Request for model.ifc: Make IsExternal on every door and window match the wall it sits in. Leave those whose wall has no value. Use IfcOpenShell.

First a look at what the model holds.

```python
import ifcopenshell
import ifcopenshell.util.element

model = ifcopenshell.open("model.ifc")
print(model.schema)
seen = {}
for e in model.by_type("IfcDoor") + model.by_type("IfcWindow"):
    if not e.FillsVoids:
        continue
    host = e.FillsVoids[0].RelatingOpeningElement.VoidsElements[0].RelatingBuildingElement
    own = ifcopenshell.util.element.get_pset(e, f"Pset_{e.is_a()[3:].removesuffix('StandardCase')}Common", "IsExternal")
    wall = ifcopenshell.util.element.get_pset(host, "Pset_WallCommon", "IsExternal")
    seen[e.is_a(), own, wall] = seen.get((e.is_a(), own, wall), 0) + 1
for (cls, own, wall), count in sorted(seen.items(), key=str):
    print(count, cls, "IsExternal:", own, "| host wall:", wall)
```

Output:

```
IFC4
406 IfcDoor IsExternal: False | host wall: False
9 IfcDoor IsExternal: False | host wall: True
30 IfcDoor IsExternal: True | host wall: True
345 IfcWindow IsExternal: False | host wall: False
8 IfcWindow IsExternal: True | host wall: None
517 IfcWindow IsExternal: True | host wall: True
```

```python
import ifcopenshell
import ifcopenshell.api.pset
import ifcopenshell.util.element

model = ifcopenshell.open("model.ifc")

count = 0
for ifc_class, pset_name in (("IfcDoor", "Pset_DoorCommon"), ("IfcWindow", "Pset_WindowCommon")):
    for e in model.by_type(ifc_class):
        if not e.FillsVoids:
            continue
        host = e.FillsVoids[0].RelatingOpeningElement.VoidsElements[0].RelatingBuildingElement
        external = ifcopenshell.util.element.get_pset(host, "Pset_WallCommon", "IsExternal")
        if external is None or ifcopenshell.util.element.get_pset(e, pset_name, "IsExternal") == external:
            continue
        pset = ifcopenshell.api.pset.add_pset(model, product=e, name=pset_name)
        ifcopenshell.api.pset.edit_pset(model, pset=pset, properties={"IsExternal": external})
        count += 1

print(count, "updated")

model.write("model_v2.ifc")
```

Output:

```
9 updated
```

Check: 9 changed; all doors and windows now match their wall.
